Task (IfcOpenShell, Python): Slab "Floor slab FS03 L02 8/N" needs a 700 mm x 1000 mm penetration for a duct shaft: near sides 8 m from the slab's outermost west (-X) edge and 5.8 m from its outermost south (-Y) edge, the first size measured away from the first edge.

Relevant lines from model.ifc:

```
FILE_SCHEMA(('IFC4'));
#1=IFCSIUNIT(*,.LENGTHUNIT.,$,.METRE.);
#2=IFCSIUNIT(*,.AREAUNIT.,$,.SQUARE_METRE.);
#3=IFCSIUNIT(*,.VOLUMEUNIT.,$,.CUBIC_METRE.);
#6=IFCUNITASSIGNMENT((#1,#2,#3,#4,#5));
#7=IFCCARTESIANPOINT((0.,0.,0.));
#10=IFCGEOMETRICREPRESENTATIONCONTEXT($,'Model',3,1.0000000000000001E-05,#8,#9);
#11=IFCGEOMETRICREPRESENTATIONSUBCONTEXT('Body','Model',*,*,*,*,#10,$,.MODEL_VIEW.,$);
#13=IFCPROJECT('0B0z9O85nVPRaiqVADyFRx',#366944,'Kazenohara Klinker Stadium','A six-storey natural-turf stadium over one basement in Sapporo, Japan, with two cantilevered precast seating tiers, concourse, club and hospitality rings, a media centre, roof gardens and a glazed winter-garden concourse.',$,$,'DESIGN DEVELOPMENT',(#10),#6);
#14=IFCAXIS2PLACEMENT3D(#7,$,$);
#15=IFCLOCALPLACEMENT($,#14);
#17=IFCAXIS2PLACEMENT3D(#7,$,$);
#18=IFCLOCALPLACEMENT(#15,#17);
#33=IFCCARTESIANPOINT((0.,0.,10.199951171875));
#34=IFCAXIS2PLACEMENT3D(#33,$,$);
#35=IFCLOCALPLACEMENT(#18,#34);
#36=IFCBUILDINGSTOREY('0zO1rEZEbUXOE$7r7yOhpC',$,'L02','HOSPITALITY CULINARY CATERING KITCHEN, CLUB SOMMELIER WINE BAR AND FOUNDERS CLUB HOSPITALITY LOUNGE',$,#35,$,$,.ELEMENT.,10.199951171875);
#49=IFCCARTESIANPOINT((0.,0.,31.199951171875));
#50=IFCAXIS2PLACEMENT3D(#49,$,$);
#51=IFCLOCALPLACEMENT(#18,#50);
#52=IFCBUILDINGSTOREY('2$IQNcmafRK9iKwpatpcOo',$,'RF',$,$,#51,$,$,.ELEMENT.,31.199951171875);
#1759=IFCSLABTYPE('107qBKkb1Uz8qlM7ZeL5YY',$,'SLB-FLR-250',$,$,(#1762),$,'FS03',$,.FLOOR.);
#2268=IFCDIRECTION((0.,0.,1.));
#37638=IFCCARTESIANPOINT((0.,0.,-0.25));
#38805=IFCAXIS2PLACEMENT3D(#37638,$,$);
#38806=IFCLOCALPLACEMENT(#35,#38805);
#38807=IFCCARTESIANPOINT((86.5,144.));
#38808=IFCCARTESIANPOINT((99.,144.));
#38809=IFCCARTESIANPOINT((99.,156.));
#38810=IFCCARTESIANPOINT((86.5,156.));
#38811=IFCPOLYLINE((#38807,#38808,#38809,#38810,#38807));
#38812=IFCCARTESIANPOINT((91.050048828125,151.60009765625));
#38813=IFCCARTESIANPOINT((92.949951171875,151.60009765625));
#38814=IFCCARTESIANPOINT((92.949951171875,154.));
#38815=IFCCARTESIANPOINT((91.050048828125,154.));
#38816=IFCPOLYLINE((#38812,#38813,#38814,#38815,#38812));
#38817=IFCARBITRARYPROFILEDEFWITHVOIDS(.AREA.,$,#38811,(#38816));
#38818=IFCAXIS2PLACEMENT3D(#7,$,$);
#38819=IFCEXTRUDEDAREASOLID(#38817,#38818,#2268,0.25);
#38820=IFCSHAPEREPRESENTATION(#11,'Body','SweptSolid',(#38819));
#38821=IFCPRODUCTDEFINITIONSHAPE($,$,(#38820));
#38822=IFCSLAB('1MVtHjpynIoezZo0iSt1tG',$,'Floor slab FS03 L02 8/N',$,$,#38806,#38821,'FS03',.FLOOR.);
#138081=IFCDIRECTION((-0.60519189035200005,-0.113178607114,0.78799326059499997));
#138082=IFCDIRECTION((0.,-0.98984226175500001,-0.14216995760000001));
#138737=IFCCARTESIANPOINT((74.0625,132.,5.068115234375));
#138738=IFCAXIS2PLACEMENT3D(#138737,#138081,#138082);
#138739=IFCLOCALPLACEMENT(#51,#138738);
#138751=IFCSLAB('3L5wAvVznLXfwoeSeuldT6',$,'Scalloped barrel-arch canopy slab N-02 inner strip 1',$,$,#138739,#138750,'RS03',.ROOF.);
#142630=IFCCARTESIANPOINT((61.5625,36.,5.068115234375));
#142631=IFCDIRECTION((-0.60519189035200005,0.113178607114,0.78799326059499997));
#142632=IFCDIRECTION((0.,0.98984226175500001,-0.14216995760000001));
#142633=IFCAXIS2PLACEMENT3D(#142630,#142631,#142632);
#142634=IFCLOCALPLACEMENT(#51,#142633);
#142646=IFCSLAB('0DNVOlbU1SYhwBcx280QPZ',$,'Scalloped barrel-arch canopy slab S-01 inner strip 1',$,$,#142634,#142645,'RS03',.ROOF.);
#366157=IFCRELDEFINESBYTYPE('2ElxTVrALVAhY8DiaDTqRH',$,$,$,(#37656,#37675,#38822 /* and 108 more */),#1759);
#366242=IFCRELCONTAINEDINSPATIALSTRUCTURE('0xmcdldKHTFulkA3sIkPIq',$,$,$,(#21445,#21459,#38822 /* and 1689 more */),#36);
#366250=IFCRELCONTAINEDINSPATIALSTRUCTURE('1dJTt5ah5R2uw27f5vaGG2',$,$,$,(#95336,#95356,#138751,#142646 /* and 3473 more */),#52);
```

```python
import numpy as np
import ifcopenshell
import ifcopenshell.api.feature
import ifcopenshell.api.geometry
import ifcopenshell.api.root
import ifcopenshell.geom
import ifcopenshell.util.placement
import ifcopenshell.util.representation
import ifcopenshell.util.shape
import ifcopenshell.util.unit

model = ifcopenshell.open("model.ifc")
unit_scale = ifcopenshell.util.unit.calculate_unit_scale(model)
settings = ifcopenshell.geom.settings()


def volume(element):
    """Net volume in cubic metres, openings subtracted."""
    shape = ifcopenshell.geom.create_shape(settings, element)
    return ifcopenshell.util.shape.get_volume(shape.geometry)


slab = model.by_guid("1MVtHjpynIoezZo0iSt1tG")
before = volume(slab)

# Extent in the slab's own axes, in metres. The edges named are its -X and -Y sides.
slab_shape = ifcopenshell.geom.create_shape(settings, slab)
vertices = ifcopenshell.util.shape.get_vertices(slab_shape.geometry)
x_min, y_min, bottom = vertices.min(axis=0)
top = vertices[:, 2].max()

opening = ifcopenshell.api.root.create_entity(model, ifc_class="IfcOpeningElement", name="Duct shaft opening", predefined_type="OPENING")
context = ifcopenshell.util.representation.get_context(model, "Model", "Body", "MODEL_VIEW")
width, depth = 0.7, 1
outline = [(0.0, 0.0), (width, 0.0), (width, depth), (0.0, depth), (0.0, 0.0)]
# Overshoot both faces by 50 mm so the cut is clean.
shape = ifcopenshell.api.geometry.add_slab_representation(
    model, context=context, depth=top - bottom + 0.1, polyline=outline
)
ifcopenshell.api.geometry.assign_representation(model, product=opening, representation=shape)

matrix = ifcopenshell.util.placement.get_local_placement(slab.ObjectPlacement)
matrix[:, 3] = matrix @ np.append(np.array([x_min + 8, y_min + 5.8, bottom - 0.05]) / unit_scale, 1.0)
ifcopenshell.api.geometry.edit_object_placement(model, product=opening, matrix=matrix, is_si=False)
ifcopenshell.api.feature.add_feature(model, feature=opening, element=slab)

after = volume(slab)

print(f"slab volume {before:.3f} -> {after:.3f} m3")

model.write("model_edited.ifc")
```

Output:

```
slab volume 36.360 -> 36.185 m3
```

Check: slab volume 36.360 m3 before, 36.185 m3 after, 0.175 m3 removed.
